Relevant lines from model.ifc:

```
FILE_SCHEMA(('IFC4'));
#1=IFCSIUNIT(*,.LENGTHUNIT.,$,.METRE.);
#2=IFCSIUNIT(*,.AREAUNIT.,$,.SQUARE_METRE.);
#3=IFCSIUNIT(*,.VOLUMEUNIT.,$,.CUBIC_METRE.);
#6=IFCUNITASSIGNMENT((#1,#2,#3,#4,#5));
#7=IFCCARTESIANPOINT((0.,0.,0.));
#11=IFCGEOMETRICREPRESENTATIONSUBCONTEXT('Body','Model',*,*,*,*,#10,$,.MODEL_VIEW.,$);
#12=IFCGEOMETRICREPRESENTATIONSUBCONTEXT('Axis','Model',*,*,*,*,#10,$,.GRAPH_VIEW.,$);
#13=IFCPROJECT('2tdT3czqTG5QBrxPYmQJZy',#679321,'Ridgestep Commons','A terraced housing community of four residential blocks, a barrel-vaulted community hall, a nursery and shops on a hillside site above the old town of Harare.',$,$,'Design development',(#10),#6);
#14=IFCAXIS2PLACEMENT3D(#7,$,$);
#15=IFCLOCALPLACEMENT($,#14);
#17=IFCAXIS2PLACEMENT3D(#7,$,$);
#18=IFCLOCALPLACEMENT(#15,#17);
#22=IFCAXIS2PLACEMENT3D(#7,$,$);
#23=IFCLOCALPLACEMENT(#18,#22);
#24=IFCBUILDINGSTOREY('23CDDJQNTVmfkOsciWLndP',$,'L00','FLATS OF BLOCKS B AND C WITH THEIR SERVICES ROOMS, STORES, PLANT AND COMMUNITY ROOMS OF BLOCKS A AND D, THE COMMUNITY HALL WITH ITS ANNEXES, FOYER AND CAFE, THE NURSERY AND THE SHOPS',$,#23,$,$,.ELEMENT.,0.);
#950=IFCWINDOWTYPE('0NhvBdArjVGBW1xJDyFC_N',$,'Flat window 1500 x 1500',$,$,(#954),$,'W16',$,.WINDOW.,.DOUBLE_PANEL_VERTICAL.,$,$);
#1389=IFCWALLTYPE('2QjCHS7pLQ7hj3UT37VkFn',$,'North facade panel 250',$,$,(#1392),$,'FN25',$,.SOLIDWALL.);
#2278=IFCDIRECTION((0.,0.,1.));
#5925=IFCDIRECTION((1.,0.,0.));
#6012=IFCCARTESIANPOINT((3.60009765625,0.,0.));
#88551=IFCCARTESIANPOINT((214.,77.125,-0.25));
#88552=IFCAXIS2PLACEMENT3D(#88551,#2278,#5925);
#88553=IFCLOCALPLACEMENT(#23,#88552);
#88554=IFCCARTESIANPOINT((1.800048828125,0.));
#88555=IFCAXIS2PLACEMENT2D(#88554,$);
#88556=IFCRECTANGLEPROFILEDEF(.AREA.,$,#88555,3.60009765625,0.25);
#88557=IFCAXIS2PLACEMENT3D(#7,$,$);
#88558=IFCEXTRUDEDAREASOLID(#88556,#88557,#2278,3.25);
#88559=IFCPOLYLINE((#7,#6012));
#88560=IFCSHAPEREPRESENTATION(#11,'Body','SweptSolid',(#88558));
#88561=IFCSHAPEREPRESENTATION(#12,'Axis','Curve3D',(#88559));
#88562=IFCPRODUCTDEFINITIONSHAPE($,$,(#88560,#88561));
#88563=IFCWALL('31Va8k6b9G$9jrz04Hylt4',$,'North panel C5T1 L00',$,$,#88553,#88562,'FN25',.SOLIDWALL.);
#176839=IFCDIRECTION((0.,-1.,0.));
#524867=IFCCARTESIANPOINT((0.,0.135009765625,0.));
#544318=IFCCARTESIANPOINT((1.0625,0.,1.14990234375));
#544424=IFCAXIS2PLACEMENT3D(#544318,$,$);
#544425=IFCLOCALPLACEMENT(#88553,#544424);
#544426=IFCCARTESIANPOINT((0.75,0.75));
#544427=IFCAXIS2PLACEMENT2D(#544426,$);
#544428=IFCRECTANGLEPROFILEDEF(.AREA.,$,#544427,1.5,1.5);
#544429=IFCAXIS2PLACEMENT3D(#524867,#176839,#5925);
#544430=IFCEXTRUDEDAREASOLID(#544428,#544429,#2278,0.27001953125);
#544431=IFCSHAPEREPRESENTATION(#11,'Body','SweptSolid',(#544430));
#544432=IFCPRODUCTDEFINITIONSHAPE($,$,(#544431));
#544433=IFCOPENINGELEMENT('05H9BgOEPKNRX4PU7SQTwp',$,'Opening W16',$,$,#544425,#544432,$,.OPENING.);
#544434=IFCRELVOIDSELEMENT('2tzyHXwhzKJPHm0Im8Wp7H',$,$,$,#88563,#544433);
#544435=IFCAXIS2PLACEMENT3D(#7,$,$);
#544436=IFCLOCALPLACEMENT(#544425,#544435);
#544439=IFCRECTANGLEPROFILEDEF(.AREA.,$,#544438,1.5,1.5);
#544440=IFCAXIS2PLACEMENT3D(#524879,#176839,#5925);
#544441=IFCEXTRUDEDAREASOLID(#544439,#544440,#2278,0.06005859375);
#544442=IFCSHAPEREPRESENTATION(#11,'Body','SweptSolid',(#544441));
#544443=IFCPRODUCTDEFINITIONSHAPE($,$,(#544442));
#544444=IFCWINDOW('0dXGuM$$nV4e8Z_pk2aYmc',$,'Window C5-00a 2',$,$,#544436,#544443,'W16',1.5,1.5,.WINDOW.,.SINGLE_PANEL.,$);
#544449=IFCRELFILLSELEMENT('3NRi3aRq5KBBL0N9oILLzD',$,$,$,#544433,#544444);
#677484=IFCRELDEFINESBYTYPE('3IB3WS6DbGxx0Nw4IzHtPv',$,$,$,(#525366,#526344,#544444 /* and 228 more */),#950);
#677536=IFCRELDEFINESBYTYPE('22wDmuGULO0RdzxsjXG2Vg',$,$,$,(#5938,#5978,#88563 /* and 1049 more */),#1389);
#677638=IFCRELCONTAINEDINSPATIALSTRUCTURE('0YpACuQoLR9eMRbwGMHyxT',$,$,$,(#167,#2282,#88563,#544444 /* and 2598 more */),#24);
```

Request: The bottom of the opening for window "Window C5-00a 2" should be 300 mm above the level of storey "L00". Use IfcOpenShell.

```python
import numpy as np
import ifcopenshell
import ifcopenshell.api.geometry
import ifcopenshell.geom
import ifcopenshell.util.element
import ifcopenshell.util.placement
import ifcopenshell.util.shape
import ifcopenshell.util.unit

model = ifcopenshell.open("model.ifc")
unit_scale = ifcopenshell.util.unit.calculate_unit_scale(model)

window = model.by_guid("0dXGuM$$nV4e8Z_pk2aYmc")
opening = window.FillsVoids[0].RelatingOpeningElement
storey = ifcopenshell.util.element.get_container(window, ifc_class="IfcBuildingStorey")
level = ifcopenshell.util.placement.get_local_placement(storey.ObjectPlacement)[2, 3]

# The opening's origin need not be at the sill, so measure its lowest point.
shape = ifcopenshell.geom.create_shape(ifcopenshell.geom.settings(), opening)
bottom = ifcopenshell.util.shape.get_shape_bottom_elevation(shape, shape.geometry) / unit_scale
dz = level + 0.3 / unit_scale - bottom

shift = np.array([0.0, 0.0, dz])
# The window is placed relative to its opening, so it follows when the opening moves.
matrix = ifcopenshell.util.placement.get_local_placement(opening.ObjectPlacement)
matrix[:3, 3] += shift
ifcopenshell.api.geometry.edit_object_placement(
    model, product=opening, matrix=matrix, is_si=False, should_transform_children=True
)

print(f"moved by {dz * unit_scale:+.3f} m")

model.write("model_updated.ifc")
```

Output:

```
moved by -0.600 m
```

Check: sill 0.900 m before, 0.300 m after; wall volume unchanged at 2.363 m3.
